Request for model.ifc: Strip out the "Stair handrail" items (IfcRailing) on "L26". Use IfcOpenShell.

First a look at what the model holds.

```python
import ifcopenshell
import ifcopenshell.util.element

model = ifcopenshell.open("model.ifc")
print(model.schema)
storey = next(s for s in model.by_type("IfcBuildingStorey") if s.Name == "L26")
railings = [e for e in ifcopenshell.util.element.get_decomposition(storey) if e.is_a("IfcRailing")]
seen = {}
for e in railings:
    element_type = ifcopenshell.util.element.get_type(e)
    name = element_type.Name if element_type not in (None, e) else None
    seen[name] = seen.get(name, 0) + 1
for name, count in sorted(seen.items(), key=str):
    print(count, "x", name)
```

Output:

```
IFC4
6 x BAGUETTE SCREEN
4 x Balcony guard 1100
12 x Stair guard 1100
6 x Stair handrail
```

```python
import ifcopenshell
import ifcopenshell.api.root
import ifcopenshell.util.element

model = ifcopenshell.open("model.ifc")

storey = next(s for s in model.by_type("IfcBuildingStorey") if s.Name == "L26")
railings = [e for e in ifcopenshell.util.element.get_decomposition(storey) if e.is_a("IfcRailing")]
targets = [e for e in railings if (t := ifcopenshell.util.element.get_type(e)) not in (None, e) and t.Name == "Stair handrail"]

for e in targets:
    ifcopenshell.api.root.remove_product(model, product=e)
print(len(targets), "removed")

model.write("model_v2.ifc")
```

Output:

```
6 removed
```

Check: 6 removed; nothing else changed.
